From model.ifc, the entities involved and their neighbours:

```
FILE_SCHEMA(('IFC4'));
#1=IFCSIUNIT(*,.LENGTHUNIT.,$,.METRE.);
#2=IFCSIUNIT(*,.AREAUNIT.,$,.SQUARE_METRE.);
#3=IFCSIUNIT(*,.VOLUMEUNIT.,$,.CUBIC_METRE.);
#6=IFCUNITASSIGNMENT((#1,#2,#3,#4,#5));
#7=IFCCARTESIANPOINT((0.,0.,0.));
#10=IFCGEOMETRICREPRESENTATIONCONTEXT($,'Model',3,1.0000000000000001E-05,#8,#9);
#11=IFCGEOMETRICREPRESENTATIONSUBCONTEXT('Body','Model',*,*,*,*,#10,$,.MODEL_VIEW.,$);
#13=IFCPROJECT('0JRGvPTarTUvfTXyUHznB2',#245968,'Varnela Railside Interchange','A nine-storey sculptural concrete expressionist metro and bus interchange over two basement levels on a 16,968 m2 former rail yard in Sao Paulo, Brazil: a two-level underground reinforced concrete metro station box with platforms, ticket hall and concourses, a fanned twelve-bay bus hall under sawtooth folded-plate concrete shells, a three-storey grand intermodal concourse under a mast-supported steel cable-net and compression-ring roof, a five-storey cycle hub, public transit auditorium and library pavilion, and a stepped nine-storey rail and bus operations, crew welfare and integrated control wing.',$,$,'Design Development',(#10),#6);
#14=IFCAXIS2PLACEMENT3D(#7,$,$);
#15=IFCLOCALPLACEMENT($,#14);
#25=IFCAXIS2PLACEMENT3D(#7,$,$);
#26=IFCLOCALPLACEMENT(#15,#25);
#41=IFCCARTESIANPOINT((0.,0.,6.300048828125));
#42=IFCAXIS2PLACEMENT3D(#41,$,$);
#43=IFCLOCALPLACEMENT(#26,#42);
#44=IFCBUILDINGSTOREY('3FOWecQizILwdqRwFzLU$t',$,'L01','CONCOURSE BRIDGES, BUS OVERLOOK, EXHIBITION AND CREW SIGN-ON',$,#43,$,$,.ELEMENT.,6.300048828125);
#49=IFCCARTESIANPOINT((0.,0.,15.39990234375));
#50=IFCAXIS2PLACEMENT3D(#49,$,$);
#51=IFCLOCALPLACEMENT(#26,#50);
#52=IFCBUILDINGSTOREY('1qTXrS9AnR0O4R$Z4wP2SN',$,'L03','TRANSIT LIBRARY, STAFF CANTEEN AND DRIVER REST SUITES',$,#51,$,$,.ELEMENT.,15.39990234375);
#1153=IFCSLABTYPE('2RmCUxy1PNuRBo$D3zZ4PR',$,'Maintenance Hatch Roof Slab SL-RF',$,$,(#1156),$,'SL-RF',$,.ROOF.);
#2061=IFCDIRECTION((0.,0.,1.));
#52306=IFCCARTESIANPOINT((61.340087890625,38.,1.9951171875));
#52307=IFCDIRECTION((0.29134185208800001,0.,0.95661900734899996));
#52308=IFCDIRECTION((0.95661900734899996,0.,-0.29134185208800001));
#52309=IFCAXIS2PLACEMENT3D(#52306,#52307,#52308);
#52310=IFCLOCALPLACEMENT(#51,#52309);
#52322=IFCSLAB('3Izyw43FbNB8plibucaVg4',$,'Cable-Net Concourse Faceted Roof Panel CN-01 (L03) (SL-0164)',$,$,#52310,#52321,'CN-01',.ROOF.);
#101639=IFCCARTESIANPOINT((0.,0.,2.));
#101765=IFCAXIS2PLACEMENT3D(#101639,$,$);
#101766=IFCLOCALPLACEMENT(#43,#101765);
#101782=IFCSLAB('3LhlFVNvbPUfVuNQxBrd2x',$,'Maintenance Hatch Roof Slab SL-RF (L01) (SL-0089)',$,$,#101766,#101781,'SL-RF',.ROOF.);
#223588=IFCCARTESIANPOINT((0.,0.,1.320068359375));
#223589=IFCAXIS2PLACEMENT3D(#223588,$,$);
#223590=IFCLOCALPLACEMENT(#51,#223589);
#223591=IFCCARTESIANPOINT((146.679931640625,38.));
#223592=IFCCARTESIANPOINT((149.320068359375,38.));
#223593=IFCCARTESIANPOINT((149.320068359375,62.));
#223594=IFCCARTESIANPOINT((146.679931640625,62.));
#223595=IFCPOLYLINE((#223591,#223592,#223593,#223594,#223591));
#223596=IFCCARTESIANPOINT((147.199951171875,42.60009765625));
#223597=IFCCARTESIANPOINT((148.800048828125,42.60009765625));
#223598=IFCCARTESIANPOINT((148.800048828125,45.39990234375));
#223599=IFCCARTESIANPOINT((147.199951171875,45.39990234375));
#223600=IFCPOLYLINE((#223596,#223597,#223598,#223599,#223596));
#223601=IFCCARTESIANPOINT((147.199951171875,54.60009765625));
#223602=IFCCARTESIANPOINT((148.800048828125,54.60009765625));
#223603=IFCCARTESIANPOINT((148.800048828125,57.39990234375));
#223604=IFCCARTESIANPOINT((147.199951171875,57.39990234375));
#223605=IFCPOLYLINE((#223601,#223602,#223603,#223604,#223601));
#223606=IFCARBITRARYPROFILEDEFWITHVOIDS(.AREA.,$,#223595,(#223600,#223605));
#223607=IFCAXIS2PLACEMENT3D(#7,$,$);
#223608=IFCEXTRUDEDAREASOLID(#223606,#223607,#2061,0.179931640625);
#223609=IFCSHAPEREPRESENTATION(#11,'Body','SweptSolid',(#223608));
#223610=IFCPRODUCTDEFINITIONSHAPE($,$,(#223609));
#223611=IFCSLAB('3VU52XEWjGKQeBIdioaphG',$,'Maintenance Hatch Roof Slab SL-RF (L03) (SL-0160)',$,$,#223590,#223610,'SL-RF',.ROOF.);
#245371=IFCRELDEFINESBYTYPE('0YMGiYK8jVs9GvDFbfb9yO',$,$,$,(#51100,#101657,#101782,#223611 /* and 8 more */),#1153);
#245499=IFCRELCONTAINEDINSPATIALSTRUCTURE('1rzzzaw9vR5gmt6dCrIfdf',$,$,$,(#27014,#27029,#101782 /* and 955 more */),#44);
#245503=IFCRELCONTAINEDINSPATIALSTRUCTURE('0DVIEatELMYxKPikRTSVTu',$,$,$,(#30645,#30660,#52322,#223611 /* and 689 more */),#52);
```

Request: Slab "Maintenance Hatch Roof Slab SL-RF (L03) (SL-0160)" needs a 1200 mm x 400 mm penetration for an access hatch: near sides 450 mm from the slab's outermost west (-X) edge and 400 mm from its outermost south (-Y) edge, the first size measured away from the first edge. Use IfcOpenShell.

```python
import numpy as np
import ifcopenshell
import ifcopenshell.api.feature
import ifcopenshell.api.geometry
import ifcopenshell.api.root
import ifcopenshell.geom
import ifcopenshell.util.placement
import ifcopenshell.util.representation
import ifcopenshell.util.shape
import ifcopenshell.util.unit

model = ifcopenshell.open("model.ifc")
unit_scale = ifcopenshell.util.unit.calculate_unit_scale(model)
settings = ifcopenshell.geom.settings()


def volume(element):
    """Net volume in cubic metres, openings subtracted."""
    shape = ifcopenshell.geom.create_shape(settings, element)
    return ifcopenshell.util.shape.get_volume(shape.geometry)


slab = model.by_guid("3VU52XEWjGKQeBIdioaphG")
before = volume(slab)

# Extent in the slab's own axes, in metres. The edges named are its -X and -Y sides.
slab_shape = ifcopenshell.geom.create_shape(settings, slab)
vertices = ifcopenshell.util.shape.get_vertices(slab_shape.geometry)
x_min, y_min, bottom = vertices.min(axis=0)
top = vertices[:, 2].max()

opening = ifcopenshell.api.root.create_entity(model, ifc_class="IfcOpeningElement", name="Access hatch opening", predefined_type="OPENING")
context = ifcopenshell.util.representation.get_context(model, "Model", "Body", "MODEL_VIEW")
width, depth = 1.2, 0.4
outline = [(0.0, 0.0), (width, 0.0), (width, depth), (0.0, depth), (0.0, 0.0)]
# Overshoot both faces by 50 mm so the cut is clean.
shape = ifcopenshell.api.geometry.add_slab_representation(
    model, context=context, depth=top - bottom + 0.1, polyline=outline
)
ifcopenshell.api.geometry.assign_representation(model, product=opening, representation=shape)

matrix = ifcopenshell.util.placement.get_local_placement(slab.ObjectPlacement)
matrix[:, 3] = matrix @ np.append(np.array([x_min + 0.45, y_min + 0.4, bottom - 0.05]) / unit_scale, 1.0)
ifcopenshell.api.geometry.edit_object_placement(model, product=opening, matrix=matrix, is_si=False)
ifcopenshell.api.feature.add_feature(model, feature=opening, element=slab)

after = volume(slab)

print(f"slab volume {before:.3f} -> {after:.3f} m3")

model.write("model-out.ifc")
```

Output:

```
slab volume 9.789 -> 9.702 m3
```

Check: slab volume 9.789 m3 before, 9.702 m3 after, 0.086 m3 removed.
